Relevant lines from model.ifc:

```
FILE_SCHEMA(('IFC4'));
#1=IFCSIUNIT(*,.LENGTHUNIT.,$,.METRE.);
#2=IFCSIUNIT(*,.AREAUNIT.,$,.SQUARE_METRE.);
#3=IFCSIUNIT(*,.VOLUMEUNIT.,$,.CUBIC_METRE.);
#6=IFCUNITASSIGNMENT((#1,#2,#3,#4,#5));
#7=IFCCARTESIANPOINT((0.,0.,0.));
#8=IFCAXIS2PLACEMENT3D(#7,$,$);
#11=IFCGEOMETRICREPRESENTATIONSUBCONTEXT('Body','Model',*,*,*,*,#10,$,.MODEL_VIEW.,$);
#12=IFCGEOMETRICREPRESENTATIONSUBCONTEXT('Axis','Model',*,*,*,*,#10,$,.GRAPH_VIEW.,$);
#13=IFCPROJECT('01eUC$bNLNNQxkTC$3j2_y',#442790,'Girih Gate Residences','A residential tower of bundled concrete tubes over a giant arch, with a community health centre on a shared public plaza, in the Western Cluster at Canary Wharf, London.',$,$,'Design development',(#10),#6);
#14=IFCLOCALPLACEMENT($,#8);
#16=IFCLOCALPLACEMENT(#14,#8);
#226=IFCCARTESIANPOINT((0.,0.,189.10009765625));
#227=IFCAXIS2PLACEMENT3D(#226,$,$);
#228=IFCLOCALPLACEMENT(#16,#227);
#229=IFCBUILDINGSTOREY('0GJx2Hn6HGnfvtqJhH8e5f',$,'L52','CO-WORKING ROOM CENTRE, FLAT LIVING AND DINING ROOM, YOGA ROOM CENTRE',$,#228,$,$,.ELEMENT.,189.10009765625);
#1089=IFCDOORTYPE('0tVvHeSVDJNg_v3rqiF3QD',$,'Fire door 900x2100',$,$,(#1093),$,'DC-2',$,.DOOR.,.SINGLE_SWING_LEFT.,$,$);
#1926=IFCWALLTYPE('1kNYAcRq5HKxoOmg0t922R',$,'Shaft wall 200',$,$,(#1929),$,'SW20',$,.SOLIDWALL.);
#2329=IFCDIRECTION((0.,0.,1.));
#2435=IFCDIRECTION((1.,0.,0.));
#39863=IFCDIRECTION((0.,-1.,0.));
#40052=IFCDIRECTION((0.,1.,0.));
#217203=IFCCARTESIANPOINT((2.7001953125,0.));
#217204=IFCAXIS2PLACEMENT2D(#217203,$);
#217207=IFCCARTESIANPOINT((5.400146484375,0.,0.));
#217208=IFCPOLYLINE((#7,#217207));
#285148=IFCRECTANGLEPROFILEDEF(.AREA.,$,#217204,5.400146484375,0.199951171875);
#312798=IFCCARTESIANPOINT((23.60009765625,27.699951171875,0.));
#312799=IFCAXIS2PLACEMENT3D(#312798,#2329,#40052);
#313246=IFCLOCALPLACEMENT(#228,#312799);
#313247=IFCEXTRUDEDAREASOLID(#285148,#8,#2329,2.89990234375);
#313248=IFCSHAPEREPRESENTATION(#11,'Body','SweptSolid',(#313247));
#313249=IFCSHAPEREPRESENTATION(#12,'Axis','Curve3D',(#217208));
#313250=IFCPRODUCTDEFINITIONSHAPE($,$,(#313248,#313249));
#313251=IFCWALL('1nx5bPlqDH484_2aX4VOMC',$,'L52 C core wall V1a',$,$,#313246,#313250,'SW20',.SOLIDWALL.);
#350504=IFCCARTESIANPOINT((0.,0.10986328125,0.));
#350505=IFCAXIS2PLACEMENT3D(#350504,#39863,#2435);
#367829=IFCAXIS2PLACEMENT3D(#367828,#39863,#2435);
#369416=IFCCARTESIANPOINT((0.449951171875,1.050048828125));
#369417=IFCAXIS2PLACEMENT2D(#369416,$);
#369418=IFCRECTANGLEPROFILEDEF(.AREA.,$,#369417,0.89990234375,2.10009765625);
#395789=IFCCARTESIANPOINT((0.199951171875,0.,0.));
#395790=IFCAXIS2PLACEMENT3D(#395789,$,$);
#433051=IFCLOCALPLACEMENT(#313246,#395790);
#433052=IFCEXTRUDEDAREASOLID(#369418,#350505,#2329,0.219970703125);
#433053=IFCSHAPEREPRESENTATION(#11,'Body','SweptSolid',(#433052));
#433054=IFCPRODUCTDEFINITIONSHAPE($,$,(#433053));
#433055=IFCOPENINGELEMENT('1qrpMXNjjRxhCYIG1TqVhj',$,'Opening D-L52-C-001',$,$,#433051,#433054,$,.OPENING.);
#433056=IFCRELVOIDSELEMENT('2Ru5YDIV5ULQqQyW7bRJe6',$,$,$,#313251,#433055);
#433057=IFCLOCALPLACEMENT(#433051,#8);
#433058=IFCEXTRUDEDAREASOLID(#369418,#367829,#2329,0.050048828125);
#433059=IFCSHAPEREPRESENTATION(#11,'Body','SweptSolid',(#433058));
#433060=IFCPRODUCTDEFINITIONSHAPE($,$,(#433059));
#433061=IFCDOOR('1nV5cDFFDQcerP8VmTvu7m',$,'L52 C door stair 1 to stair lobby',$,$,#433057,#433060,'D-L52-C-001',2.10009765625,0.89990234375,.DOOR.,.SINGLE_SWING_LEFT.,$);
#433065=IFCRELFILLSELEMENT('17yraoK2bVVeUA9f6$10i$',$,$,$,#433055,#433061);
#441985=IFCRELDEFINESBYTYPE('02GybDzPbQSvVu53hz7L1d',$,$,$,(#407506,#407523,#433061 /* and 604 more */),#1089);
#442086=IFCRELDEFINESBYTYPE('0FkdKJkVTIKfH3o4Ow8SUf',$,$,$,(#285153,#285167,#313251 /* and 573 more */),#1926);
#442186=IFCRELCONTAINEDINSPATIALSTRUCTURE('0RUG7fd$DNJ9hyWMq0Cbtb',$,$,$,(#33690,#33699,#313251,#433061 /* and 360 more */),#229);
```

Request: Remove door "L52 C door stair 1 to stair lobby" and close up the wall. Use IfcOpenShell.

```python
import ifcopenshell
import ifcopenshell.api.feature
import ifcopenshell.api.root
import ifcopenshell.geom
import ifcopenshell.util.shape

model = ifcopenshell.open("model.ifc")
settings = ifcopenshell.geom.settings()


def volume(element):
    """Net volume in cubic metres, openings subtracted."""
    shape = ifcopenshell.geom.create_shape(settings, element)
    return ifcopenshell.util.shape.get_volume(shape.geometry)


door = model.by_id(433061)
opening = door.FillsVoids[0].RelatingOpeningElement
wall = opening.VoidsElements[0].RelatingBuildingElement
before = volume(wall)

ifcopenshell.api.root.remove_product(model, product=door)
ifcopenshell.api.feature.remove_feature(model, feature=opening)

after = volume(wall)

print(f"wall volume {before:.3f} -> {after:.3f} m3")

model.write("model_updated.ifc")
```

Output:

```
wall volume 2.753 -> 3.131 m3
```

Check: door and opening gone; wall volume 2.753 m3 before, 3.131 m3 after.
